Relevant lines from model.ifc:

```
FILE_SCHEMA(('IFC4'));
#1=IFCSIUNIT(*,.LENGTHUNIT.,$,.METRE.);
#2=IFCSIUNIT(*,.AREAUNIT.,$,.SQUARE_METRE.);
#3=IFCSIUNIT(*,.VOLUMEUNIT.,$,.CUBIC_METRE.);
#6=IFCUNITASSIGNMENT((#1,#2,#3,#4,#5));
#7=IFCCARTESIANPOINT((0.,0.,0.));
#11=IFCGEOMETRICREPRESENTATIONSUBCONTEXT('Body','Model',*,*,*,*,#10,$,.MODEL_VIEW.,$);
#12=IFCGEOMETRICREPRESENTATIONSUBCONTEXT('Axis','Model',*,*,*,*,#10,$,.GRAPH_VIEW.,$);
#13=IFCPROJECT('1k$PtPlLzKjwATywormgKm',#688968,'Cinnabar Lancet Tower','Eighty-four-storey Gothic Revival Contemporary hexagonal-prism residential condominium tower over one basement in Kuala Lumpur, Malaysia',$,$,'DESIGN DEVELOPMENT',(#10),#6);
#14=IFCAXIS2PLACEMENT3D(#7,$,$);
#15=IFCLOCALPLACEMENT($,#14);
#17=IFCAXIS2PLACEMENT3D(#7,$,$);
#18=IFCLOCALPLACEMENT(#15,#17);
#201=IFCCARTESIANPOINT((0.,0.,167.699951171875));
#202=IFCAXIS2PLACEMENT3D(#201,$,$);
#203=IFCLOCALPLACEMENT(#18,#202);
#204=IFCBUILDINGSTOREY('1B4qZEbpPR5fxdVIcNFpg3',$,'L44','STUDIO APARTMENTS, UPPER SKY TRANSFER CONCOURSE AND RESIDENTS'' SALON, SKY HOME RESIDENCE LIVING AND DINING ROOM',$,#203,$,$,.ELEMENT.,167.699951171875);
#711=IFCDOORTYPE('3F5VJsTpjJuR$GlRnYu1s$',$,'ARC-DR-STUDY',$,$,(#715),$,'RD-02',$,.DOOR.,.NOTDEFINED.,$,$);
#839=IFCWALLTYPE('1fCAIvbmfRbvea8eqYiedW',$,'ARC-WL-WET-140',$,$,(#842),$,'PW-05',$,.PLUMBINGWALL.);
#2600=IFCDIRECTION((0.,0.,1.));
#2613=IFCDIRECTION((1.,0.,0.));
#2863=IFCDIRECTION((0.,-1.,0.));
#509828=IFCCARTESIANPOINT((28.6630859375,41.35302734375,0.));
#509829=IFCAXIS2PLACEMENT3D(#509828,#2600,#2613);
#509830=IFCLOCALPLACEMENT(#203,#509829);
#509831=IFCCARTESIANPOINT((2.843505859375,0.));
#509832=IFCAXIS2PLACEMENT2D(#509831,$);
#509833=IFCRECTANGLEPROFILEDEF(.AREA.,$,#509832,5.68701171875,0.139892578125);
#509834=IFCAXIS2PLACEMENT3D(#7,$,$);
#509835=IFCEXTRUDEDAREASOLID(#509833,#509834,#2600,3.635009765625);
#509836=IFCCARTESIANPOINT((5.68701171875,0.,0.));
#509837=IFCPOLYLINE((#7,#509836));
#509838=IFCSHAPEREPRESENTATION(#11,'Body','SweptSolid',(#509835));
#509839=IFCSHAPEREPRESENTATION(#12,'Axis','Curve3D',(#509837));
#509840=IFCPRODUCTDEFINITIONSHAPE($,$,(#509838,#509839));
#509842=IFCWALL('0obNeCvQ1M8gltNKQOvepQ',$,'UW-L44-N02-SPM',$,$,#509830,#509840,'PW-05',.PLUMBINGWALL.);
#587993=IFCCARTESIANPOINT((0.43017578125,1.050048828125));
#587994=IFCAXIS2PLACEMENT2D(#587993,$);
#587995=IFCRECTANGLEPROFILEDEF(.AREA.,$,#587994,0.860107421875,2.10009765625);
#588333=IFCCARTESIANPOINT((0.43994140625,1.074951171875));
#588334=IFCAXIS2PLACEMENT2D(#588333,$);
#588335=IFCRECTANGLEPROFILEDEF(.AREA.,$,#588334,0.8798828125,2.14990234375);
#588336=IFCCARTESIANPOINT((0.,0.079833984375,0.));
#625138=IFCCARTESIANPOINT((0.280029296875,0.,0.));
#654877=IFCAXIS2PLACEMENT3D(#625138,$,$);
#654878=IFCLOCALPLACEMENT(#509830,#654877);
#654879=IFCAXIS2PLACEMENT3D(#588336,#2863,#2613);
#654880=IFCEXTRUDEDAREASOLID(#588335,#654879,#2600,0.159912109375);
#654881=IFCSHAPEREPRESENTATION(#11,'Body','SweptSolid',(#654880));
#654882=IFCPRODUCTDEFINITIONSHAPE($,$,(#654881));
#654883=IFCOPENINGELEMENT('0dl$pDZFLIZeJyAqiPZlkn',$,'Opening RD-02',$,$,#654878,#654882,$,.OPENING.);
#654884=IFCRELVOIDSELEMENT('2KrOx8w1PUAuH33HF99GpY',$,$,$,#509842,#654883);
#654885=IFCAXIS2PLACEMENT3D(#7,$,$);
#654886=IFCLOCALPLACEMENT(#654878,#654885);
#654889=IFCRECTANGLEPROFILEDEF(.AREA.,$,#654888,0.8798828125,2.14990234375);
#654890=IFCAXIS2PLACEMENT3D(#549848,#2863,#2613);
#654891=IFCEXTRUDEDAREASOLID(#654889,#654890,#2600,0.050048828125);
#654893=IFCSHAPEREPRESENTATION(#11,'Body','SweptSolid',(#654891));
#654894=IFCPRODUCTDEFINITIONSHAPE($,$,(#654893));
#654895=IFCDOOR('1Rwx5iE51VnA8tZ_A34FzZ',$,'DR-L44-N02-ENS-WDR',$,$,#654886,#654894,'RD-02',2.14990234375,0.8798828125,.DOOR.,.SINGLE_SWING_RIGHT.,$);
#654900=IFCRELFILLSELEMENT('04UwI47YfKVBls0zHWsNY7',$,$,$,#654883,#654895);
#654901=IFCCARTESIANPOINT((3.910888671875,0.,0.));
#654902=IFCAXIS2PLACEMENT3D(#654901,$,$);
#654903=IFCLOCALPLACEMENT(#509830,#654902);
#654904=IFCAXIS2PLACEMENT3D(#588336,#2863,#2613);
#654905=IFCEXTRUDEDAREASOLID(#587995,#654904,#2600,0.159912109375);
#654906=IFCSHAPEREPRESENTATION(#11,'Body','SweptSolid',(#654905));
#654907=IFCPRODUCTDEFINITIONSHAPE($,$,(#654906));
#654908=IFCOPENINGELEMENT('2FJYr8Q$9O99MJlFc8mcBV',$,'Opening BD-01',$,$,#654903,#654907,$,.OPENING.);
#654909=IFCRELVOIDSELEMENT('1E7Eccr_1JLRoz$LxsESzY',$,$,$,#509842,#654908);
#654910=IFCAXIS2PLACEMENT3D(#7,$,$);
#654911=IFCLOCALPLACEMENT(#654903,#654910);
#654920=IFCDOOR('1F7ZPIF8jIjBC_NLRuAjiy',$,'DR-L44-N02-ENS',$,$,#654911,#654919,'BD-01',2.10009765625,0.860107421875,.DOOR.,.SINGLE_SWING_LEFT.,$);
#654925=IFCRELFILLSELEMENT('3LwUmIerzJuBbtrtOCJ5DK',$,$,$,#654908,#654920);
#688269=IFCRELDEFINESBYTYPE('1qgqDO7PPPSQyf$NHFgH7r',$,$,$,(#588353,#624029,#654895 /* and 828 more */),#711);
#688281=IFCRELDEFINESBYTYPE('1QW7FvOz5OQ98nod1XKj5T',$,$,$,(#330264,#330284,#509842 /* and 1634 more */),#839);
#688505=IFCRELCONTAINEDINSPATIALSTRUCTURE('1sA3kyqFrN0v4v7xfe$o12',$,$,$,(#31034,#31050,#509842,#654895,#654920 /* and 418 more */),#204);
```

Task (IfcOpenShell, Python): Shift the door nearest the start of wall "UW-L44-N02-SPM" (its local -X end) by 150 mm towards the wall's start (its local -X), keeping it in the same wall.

```python
import ifcopenshell
import ifcopenshell.api.geometry
import ifcopenshell.util.placement
import ifcopenshell.util.unit

model = ifcopenshell.open("model.ifc")
unit_scale = ifcopenshell.util.unit.calculate_unit_scale(model)

door = model.by_guid("1Rwx5iE51VnA8tZ_A34FzZ")
opening = door.FillsVoids[0].RelatingOpeningElement
wall = opening.VoidsElements[0].RelatingBuildingElement

wall_matrix = ifcopenshell.util.placement.get_local_placement(wall.ObjectPlacement)
shift = wall_matrix[:3, 0] * -0.15 / unit_scale
before = ifcopenshell.util.placement.get_local_placement(door.ObjectPlacement)[:3, 3].copy()

# The door is placed relative to its opening, so it follows when the opening moves.
matrix = ifcopenshell.util.placement.get_local_placement(opening.ObjectPlacement)
matrix[:3, 3] += shift
ifcopenshell.api.geometry.edit_object_placement(
    model, product=opening, matrix=matrix, is_si=False, should_transform_children=True
)

after = ifcopenshell.util.placement.get_local_placement(door.ObjectPlacement)[:3, 3]
print("door moved by", (after - before).round(3) + 0.0)

model.write("model_rev.ifc")
```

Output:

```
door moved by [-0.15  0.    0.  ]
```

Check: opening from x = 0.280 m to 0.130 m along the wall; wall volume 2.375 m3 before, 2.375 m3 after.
